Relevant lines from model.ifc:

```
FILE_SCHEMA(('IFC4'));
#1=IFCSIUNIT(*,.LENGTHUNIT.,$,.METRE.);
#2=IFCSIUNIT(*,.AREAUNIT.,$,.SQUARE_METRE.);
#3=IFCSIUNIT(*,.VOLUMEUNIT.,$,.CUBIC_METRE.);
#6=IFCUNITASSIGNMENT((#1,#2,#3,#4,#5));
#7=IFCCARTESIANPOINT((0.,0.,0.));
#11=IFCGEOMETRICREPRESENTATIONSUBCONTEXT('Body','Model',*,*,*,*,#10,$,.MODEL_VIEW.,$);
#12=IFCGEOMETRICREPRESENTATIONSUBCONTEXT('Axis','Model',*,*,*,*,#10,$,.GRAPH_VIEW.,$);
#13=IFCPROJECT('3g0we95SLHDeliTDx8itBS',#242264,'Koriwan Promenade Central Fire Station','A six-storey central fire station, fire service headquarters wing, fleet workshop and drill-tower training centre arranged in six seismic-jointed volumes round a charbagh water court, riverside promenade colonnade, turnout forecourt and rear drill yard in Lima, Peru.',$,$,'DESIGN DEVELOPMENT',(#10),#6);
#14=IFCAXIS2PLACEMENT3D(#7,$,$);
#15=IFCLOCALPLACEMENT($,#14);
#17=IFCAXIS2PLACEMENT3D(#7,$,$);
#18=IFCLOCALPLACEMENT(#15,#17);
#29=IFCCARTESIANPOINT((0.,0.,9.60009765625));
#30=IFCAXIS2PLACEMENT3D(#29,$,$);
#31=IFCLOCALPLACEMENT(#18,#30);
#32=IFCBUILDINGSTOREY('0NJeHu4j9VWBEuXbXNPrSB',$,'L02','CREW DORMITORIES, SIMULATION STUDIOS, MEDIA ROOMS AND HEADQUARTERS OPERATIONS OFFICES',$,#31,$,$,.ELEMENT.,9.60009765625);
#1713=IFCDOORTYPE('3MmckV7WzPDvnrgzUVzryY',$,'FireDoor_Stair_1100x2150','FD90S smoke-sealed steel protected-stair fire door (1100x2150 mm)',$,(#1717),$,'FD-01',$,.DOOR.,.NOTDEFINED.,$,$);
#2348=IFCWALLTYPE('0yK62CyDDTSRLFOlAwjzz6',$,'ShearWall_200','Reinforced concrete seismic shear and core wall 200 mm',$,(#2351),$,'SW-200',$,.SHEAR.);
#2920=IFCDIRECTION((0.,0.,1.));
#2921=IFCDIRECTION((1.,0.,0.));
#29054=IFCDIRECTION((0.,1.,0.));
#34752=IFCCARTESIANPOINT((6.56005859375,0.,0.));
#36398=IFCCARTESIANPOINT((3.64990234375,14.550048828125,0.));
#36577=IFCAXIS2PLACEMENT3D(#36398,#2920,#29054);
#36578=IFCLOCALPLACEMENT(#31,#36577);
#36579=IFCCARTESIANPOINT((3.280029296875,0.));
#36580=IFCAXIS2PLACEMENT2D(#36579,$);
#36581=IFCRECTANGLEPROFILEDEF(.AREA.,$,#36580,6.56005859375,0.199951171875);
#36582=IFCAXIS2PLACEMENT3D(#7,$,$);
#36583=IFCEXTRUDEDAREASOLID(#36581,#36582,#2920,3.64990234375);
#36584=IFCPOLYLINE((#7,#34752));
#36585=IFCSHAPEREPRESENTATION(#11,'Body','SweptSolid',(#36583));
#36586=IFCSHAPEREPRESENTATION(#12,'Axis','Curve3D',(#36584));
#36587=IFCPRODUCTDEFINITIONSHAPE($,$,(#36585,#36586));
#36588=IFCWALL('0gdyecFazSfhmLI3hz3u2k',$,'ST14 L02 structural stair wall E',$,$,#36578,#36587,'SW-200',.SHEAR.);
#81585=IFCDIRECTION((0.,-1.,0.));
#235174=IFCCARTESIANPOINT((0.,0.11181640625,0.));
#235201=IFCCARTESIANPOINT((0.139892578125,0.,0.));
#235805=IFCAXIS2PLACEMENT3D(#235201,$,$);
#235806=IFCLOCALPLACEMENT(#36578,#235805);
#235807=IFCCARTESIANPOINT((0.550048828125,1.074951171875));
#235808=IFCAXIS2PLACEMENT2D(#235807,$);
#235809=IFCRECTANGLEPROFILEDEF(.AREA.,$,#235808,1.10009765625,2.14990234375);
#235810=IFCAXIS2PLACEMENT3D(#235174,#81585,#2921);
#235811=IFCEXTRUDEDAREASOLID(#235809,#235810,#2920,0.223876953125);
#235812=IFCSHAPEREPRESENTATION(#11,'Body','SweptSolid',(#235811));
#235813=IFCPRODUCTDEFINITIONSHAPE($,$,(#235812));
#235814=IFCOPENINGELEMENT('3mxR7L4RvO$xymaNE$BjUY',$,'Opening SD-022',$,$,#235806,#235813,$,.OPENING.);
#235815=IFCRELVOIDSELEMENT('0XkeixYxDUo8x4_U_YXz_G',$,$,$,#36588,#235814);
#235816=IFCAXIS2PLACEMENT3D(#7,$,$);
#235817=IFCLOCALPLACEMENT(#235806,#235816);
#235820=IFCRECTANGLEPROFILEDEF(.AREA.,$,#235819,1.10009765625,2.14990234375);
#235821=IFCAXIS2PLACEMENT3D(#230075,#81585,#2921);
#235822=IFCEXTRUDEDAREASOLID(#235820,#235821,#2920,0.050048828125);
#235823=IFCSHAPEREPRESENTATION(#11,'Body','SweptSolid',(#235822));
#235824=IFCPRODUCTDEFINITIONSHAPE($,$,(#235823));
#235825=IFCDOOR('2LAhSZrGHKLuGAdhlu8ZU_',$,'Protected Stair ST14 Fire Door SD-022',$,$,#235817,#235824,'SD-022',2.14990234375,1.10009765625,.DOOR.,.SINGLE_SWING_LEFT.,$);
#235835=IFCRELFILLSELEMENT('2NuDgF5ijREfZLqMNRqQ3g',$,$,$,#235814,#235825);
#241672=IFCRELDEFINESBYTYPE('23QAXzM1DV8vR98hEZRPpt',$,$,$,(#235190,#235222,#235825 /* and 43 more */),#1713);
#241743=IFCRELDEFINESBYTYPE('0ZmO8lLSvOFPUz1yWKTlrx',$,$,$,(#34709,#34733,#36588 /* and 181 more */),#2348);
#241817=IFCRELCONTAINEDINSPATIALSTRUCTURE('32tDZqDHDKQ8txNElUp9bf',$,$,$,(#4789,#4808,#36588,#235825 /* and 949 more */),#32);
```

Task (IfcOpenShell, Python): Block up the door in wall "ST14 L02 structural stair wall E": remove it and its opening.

```python
import ifcopenshell
import ifcopenshell.api.feature
import ifcopenshell.api.root
import ifcopenshell.geom
import ifcopenshell.util.shape

model = ifcopenshell.open("model.ifc")
settings = ifcopenshell.geom.settings()


def volume(element):
    """Net volume in cubic metres, openings subtracted."""
    shape = ifcopenshell.geom.create_shape(settings, element)
    return ifcopenshell.util.shape.get_volume(shape.geometry)


door = model.by_guid("2LAhSZrGHKLuGAdhlu8ZU_")
opening = door.FillsVoids[0].RelatingOpeningElement
wall = opening.VoidsElements[0].RelatingBuildingElement
before = volume(wall)

ifcopenshell.api.root.remove_product(model, product=door)
ifcopenshell.api.feature.remove_feature(model, feature=opening)

after = volume(wall)

print(f"wall volume {before:.3f} -> {after:.3f} m3")

model.write("model-out.ifc")
```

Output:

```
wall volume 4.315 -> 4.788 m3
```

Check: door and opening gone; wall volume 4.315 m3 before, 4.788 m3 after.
